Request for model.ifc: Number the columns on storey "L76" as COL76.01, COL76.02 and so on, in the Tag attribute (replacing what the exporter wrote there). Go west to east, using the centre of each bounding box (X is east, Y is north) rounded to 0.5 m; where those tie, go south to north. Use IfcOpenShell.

First a look at what the model holds.

```python
import ifcopenshell
import ifcopenshell.util.element
import ifcopenshell.util.placement

model = ifcopenshell.open("model.ifc")
print(model.schema)
storey = next(s for s in model.by_type("IfcBuildingStorey") if s.Name == "L76")
columns = [e for e in ifcopenshell.util.element.get_decomposition(storey) if e.is_a("IfcColumn")]
for e in sorted(columns, key=lambda e: e.id()):
    origin = ifcopenshell.util.placement.get_local_placement(e.ObjectPlacement)[:3, 3]
    print(e.id(), e.Tag, e.Name, origin.round(2) + 0.0, sep=" | ")
```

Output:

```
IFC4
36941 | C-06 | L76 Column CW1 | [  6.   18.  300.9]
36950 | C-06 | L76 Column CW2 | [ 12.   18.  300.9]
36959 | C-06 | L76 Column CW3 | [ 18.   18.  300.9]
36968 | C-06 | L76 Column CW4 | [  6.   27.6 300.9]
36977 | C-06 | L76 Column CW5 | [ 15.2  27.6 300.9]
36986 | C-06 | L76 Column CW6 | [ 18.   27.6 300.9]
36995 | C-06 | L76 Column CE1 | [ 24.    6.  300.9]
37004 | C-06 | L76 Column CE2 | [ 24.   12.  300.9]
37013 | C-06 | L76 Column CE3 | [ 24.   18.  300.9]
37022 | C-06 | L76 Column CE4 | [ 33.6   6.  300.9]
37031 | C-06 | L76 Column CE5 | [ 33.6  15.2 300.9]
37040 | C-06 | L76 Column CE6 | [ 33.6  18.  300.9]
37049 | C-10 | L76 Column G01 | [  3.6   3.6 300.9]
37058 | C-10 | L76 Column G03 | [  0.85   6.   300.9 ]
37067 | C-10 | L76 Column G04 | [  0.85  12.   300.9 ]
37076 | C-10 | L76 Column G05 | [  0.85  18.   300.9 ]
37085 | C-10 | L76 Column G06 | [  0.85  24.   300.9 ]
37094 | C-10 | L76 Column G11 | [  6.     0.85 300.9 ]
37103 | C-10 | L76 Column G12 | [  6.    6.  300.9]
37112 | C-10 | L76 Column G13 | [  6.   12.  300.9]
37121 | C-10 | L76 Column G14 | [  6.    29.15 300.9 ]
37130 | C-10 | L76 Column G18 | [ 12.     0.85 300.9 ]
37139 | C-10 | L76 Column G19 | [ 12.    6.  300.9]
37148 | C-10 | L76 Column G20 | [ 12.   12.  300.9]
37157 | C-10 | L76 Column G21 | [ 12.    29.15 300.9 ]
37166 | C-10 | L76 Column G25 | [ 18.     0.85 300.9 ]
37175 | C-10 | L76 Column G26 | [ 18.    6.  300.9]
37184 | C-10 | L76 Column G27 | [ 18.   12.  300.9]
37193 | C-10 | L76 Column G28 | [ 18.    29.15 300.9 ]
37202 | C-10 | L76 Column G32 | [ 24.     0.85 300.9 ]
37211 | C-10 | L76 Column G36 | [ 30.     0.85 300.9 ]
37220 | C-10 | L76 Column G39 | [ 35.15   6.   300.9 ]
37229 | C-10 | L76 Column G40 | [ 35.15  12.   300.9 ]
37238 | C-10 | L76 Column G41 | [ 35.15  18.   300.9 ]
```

```python
import ifcopenshell
import ifcopenshell.geom
import ifcopenshell.util.element
import ifcopenshell.util.shape

model = ifcopenshell.open("model.ifc")
settings = ifcopenshell.geom.settings()
settings.set("use-world-coords", True)


def centre(element):
    shape = ifcopenshell.geom.create_shape(settings, element)
    return ifcopenshell.util.shape.get_bbox_centroid(shape.geometry)


storey = next(s for s in model.by_type("IfcBuildingStorey") if s.Name == "L76")
columns = [e for e in ifcopenshell.util.element.get_decomposition(storey) if e.is_a("IfcColumn")]

# Insertion points can sit at a corner or the storey origin, so sort by the geometry (in metres).
centres = {e: centre(e) for e in columns}
columns.sort(key=lambda e: (round(centres[e][0] / 0.5), centres[e][1]))

for i, e in enumerate(columns, start=1):
    number = f"COL76.{i:02d}"
    e.Tag = number
    print(e.id(), number)

model.write("model_v2.ifc")
```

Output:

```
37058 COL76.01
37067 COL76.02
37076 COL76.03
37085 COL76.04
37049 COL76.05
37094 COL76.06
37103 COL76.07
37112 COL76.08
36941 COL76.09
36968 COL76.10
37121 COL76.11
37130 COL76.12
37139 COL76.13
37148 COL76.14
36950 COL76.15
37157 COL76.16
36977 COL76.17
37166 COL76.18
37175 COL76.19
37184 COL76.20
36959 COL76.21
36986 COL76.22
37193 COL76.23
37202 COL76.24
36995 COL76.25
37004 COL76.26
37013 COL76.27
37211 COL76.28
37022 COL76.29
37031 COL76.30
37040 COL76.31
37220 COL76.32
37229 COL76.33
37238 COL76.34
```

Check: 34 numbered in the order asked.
